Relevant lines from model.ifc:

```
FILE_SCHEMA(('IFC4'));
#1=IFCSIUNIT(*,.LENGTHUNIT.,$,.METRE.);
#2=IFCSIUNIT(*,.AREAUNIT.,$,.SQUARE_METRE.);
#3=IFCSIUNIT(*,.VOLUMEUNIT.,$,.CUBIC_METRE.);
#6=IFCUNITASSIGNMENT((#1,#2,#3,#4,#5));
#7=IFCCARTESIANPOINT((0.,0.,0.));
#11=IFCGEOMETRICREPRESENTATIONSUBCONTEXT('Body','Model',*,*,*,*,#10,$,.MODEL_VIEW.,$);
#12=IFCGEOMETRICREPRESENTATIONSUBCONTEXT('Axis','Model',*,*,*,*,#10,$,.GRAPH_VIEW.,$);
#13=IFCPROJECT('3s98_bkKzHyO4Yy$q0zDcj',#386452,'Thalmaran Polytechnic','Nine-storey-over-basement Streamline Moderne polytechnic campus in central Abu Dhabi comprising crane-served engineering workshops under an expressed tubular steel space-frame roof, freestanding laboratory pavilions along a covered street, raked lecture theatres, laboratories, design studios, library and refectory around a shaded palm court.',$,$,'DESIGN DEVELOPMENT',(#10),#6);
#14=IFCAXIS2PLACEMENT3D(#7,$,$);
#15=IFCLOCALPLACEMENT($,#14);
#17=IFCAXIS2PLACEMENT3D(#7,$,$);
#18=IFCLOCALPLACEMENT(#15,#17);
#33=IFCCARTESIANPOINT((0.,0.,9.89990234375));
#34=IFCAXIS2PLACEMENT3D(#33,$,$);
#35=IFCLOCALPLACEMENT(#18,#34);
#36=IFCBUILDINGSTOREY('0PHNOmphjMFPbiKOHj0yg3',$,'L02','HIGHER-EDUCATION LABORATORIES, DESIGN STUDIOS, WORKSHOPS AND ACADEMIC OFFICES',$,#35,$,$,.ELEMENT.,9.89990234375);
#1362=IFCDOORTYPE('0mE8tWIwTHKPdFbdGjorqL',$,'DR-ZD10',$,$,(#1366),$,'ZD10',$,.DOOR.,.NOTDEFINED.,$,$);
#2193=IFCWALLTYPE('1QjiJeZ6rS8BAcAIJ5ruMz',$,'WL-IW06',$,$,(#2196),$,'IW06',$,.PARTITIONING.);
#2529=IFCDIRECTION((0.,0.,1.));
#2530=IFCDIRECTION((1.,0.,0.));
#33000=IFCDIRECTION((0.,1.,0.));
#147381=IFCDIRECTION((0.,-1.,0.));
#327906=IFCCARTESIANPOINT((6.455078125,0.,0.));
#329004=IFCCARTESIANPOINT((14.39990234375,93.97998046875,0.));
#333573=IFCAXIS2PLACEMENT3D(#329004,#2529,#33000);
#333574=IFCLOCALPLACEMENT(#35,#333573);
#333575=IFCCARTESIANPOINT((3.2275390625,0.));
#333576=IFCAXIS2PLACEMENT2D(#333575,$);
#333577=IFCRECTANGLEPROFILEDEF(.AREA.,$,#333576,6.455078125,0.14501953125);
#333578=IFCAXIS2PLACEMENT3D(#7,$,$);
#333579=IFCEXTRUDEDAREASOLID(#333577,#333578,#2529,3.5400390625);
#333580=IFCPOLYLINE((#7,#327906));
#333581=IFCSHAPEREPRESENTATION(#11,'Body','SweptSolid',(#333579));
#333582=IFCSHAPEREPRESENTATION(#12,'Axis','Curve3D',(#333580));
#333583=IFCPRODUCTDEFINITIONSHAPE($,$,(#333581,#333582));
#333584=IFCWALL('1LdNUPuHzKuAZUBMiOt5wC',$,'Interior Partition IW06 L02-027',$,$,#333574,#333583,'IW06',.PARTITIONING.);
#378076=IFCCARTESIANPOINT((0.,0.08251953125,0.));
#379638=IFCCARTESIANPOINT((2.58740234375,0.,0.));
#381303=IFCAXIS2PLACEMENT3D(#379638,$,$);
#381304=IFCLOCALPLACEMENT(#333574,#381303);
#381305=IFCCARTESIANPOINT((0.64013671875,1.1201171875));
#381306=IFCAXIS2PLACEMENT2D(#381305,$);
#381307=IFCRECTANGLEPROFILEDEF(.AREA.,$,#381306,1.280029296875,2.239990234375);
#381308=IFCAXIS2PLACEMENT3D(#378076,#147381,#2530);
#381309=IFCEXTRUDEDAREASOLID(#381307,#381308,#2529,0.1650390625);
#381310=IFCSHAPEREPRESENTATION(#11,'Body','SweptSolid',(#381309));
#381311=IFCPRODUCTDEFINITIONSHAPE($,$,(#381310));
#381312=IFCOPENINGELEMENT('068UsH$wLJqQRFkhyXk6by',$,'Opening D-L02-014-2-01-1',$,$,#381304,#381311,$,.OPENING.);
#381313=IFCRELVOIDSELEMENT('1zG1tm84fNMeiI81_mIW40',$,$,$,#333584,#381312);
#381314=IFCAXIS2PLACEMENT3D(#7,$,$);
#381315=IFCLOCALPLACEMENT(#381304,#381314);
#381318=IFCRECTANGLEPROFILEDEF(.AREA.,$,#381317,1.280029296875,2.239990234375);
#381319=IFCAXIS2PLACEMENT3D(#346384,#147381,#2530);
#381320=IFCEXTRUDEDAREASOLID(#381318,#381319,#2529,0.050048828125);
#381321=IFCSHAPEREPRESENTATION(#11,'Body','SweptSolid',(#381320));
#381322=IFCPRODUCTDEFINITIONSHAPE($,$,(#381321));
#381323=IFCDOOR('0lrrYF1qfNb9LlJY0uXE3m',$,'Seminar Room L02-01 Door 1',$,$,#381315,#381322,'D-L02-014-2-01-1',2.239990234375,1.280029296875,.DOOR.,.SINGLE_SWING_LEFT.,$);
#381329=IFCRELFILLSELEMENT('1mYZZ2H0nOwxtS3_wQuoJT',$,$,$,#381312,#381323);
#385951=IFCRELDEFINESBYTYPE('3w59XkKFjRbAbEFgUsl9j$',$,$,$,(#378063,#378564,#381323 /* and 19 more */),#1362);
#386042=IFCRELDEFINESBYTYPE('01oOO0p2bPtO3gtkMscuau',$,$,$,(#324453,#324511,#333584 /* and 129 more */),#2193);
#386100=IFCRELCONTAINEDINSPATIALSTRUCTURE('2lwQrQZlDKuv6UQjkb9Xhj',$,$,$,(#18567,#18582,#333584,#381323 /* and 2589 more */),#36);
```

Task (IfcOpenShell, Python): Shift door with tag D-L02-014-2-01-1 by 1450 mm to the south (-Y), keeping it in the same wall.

```python
import ifcopenshell
import ifcopenshell.api.geometry
import ifcopenshell.util.placement
import ifcopenshell.util.unit

model = ifcopenshell.open("model.ifc")
unit_scale = ifcopenshell.util.unit.calculate_unit_scale(model)

door = model.by_guid("0lrrYF1qfNb9LlJY0uXE3m")
opening = door.FillsVoids[0].RelatingOpeningElement
wall = opening.VoidsElements[0].RelatingBuildingElement

wall_matrix = ifcopenshell.util.placement.get_local_placement(wall.ObjectPlacement)
shift = wall_matrix[:3, 0] * -1.45 / unit_scale
before = ifcopenshell.util.placement.get_local_placement(door.ObjectPlacement)[:3, 3].copy()

# The door is placed relative to its opening, so it follows when the opening moves.
matrix = ifcopenshell.util.placement.get_local_placement(opening.ObjectPlacement)
matrix[:3, 3] += shift
ifcopenshell.api.geometry.edit_object_placement(
    model, product=opening, matrix=matrix, is_si=False, should_transform_children=True
)

after = ifcopenshell.util.placement.get_local_placement(door.ObjectPlacement)[:3, 3]
print("door moved by", (after - before).round(3) + 0.0)

model.write("model_rev.ifc")
```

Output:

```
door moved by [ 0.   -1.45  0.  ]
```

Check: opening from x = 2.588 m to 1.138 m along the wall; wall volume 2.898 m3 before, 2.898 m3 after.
